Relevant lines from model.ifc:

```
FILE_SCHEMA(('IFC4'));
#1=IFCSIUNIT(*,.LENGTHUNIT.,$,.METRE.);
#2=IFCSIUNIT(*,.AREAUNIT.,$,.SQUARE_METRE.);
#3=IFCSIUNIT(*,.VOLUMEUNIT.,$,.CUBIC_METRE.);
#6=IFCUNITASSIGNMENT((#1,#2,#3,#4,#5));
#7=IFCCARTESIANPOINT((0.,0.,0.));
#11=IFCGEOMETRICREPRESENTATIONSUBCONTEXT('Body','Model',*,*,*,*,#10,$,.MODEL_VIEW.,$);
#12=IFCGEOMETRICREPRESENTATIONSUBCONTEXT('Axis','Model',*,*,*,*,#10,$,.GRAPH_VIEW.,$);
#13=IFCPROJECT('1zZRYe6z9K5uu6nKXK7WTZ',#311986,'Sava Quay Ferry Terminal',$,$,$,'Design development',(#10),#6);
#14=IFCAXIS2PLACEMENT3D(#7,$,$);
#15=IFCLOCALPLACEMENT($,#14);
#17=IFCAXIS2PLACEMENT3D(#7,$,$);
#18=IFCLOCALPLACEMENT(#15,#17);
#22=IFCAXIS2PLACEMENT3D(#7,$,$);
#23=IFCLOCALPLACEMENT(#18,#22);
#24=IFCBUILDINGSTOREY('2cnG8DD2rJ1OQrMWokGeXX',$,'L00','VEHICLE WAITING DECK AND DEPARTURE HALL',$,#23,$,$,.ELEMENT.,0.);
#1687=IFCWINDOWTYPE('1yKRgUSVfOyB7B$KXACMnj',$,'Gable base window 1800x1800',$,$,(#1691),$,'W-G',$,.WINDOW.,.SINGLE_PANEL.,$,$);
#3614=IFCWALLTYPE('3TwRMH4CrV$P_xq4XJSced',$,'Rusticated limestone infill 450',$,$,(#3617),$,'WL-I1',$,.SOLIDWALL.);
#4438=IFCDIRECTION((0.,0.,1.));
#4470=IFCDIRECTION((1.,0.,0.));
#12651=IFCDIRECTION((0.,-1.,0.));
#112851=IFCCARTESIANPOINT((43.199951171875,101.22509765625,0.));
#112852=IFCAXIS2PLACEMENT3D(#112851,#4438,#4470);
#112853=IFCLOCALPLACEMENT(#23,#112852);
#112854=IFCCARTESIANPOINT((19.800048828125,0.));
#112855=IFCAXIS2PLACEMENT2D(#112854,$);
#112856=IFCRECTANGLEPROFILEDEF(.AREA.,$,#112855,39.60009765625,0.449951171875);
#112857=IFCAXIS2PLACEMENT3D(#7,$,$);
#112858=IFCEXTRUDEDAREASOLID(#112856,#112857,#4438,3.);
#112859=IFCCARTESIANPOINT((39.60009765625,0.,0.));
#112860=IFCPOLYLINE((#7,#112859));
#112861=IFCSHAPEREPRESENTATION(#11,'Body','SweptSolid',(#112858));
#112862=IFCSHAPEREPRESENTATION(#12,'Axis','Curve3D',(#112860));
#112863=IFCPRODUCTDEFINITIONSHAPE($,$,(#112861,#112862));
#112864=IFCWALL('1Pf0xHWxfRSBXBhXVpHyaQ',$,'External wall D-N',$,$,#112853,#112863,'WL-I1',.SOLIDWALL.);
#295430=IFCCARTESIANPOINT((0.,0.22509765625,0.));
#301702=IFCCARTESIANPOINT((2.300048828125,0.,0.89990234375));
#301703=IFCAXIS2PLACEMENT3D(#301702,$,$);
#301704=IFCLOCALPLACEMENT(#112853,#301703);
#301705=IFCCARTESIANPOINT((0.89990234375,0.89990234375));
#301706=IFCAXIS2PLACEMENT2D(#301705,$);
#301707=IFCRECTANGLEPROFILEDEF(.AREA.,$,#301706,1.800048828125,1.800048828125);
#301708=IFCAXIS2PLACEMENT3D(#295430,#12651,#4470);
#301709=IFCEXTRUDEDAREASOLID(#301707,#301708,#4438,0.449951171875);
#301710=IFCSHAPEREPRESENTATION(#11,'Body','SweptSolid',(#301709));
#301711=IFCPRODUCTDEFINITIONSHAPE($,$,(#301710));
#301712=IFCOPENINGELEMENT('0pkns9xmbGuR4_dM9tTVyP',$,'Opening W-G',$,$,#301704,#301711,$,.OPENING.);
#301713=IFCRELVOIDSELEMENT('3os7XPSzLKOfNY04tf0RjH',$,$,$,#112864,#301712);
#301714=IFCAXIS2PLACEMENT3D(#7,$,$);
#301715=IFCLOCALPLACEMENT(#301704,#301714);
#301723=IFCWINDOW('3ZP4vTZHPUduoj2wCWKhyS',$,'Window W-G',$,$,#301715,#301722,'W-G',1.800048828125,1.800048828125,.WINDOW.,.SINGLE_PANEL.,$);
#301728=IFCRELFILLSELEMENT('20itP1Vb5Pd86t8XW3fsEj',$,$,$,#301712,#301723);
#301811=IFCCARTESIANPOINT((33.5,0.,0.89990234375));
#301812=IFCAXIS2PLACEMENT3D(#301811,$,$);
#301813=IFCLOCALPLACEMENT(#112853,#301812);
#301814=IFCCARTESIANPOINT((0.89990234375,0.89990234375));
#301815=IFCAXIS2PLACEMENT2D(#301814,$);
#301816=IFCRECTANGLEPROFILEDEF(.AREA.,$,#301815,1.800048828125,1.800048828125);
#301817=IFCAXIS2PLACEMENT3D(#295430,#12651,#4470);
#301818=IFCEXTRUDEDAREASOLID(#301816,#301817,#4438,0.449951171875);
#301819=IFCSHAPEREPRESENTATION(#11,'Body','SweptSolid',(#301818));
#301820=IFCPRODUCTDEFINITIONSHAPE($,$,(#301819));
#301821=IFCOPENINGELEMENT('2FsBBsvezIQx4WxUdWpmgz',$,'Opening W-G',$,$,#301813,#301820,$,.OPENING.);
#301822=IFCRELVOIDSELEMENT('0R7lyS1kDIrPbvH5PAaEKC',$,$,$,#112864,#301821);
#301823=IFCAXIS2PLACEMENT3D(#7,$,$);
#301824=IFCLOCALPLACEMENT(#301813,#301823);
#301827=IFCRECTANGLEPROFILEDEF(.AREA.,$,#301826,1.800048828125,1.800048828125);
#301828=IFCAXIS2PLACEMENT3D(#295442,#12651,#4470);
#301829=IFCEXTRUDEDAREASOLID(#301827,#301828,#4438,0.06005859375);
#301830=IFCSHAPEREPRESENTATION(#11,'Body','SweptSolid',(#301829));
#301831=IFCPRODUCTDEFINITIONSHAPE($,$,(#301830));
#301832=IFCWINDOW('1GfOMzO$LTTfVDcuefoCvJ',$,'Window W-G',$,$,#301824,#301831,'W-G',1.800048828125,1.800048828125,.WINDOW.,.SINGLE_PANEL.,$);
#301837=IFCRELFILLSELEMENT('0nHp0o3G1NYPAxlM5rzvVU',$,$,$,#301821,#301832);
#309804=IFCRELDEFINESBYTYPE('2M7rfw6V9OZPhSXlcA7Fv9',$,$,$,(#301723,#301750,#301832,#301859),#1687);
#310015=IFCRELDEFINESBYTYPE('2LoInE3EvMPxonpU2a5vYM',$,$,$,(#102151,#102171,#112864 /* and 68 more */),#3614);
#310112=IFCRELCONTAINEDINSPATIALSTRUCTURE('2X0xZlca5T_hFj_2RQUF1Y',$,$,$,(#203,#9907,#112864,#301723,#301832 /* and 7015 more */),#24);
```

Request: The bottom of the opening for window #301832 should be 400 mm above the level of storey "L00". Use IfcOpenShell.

```python
import numpy as np
import ifcopenshell
import ifcopenshell.api.geometry
import ifcopenshell.geom
import ifcopenshell.util.element
import ifcopenshell.util.placement
import ifcopenshell.util.shape
import ifcopenshell.util.unit

model = ifcopenshell.open("model.ifc")
unit_scale = ifcopenshell.util.unit.calculate_unit_scale(model)

window = model.by_guid("1GfOMzO$LTTfVDcuefoCvJ")
opening = window.FillsVoids[0].RelatingOpeningElement
storey = ifcopenshell.util.element.get_container(window, ifc_class="IfcBuildingStorey")
level = ifcopenshell.util.placement.get_local_placement(storey.ObjectPlacement)[2, 3]

# The opening's origin need not be at the sill, so measure its lowest point.
shape = ifcopenshell.geom.create_shape(ifcopenshell.geom.settings(), opening)
bottom = ifcopenshell.util.shape.get_shape_bottom_elevation(shape, shape.geometry) / unit_scale
dz = level + 0.4 / unit_scale - bottom

shift = np.array([0.0, 0.0, dz])
# The window is placed relative to its opening, so it follows when the opening moves.
matrix = ifcopenshell.util.placement.get_local_placement(opening.ObjectPlacement)
matrix[:3, 3] += shift
ifcopenshell.api.geometry.edit_object_placement(
    model, product=opening, matrix=matrix, is_si=False, should_transform_children=True
)

print(f"moved by {dz * unit_scale:+.3f} m")

model.write("model-out.ifc")
```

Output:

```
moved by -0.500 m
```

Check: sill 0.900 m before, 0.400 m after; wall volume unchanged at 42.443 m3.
